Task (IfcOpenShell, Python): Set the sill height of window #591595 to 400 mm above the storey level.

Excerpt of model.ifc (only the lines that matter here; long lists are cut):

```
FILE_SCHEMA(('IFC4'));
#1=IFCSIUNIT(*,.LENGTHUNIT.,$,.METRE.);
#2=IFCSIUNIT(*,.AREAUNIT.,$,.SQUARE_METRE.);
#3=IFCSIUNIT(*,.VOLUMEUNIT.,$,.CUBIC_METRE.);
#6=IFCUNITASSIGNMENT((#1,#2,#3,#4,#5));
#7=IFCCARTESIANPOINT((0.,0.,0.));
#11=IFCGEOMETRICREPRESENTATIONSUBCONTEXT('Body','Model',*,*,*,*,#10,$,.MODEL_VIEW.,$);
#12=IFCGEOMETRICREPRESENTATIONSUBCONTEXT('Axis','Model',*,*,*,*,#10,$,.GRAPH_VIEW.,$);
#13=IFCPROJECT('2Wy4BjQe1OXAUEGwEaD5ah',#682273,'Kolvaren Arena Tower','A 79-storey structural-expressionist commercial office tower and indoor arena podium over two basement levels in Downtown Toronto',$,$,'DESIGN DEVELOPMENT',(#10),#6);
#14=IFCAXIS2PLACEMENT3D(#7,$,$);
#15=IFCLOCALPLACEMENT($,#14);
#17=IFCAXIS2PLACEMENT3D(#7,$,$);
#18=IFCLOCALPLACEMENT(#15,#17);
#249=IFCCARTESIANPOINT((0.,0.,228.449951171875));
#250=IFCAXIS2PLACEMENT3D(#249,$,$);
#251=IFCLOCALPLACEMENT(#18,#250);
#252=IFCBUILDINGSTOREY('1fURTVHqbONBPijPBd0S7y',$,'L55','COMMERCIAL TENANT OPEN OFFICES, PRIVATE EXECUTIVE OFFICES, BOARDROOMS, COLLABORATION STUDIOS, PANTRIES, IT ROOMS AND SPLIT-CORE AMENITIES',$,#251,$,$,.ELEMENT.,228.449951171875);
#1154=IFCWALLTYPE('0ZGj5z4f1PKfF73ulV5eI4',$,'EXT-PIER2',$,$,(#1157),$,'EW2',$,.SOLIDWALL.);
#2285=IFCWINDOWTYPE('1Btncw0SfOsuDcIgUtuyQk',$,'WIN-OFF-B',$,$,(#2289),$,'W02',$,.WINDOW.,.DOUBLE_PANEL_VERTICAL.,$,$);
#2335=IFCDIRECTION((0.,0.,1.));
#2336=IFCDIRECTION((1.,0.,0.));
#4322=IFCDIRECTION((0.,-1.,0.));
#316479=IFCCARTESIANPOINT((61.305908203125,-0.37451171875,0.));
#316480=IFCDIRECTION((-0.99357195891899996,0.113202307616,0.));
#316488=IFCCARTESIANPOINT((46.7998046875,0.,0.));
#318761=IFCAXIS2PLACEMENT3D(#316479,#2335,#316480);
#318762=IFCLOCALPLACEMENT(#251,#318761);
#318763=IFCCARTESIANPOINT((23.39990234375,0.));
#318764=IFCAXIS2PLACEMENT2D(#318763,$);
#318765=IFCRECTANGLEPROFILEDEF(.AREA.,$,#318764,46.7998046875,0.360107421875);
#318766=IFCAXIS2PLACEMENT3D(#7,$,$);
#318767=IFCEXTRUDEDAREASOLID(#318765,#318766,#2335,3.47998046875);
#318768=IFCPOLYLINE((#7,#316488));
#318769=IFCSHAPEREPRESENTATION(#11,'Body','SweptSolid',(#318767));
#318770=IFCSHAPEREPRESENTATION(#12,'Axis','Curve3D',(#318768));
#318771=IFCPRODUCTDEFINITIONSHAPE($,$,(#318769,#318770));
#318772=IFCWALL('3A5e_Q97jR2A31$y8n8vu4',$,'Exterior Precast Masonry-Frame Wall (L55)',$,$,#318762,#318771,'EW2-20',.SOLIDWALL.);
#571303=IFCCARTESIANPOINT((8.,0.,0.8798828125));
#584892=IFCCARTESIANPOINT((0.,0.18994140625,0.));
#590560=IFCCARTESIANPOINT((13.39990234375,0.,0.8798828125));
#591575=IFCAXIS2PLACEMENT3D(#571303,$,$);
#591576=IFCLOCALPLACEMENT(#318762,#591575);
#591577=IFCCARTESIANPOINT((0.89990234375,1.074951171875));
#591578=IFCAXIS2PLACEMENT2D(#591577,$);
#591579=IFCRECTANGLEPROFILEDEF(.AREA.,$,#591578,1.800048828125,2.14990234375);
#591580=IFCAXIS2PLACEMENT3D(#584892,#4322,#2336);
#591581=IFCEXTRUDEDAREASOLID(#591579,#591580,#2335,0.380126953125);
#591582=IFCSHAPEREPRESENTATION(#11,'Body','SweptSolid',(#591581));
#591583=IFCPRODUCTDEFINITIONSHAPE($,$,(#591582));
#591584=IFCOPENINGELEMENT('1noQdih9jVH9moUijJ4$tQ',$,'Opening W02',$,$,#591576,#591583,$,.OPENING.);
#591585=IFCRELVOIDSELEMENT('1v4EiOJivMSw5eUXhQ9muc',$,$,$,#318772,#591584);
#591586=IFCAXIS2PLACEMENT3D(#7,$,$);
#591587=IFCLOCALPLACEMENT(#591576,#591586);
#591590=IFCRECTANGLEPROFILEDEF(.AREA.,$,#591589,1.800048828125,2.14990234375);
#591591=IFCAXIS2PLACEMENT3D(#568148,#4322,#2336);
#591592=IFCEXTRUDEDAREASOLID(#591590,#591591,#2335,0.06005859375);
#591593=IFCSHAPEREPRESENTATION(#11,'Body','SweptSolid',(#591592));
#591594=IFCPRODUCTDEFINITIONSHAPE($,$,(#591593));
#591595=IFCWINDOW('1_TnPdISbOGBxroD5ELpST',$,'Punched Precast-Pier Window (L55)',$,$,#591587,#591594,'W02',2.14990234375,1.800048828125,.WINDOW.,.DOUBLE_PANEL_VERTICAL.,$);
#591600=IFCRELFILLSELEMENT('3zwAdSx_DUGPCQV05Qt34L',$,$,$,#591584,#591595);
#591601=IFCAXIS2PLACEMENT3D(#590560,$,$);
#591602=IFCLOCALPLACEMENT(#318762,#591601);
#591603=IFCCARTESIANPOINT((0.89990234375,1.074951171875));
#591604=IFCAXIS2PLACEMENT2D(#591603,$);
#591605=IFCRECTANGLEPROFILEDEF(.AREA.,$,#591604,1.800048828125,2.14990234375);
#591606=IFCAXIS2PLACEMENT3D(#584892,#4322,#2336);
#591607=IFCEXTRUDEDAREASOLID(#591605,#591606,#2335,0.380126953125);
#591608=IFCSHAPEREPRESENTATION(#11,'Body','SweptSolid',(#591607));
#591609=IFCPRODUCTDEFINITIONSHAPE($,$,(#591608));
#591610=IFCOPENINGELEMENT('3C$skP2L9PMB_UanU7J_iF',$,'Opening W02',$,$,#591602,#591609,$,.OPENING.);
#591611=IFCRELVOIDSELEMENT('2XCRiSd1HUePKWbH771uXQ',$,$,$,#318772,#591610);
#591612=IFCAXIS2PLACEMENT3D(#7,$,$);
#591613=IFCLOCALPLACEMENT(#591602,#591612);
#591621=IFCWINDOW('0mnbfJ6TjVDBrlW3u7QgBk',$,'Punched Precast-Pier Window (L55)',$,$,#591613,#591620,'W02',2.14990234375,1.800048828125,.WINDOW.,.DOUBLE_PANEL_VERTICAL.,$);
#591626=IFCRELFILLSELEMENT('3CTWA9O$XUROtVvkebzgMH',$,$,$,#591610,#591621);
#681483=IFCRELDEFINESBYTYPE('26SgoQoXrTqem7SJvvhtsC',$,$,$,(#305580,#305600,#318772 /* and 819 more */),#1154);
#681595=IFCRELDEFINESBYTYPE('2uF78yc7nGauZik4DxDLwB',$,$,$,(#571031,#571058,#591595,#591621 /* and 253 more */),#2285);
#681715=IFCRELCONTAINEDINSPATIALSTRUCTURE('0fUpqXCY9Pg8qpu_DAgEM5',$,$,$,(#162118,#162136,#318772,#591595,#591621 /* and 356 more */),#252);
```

```python
import numpy as np
import ifcopenshell
import ifcopenshell.api.geometry
import ifcopenshell.geom
import ifcopenshell.util.element
import ifcopenshell.util.placement
import ifcopenshell.util.shape
import ifcopenshell.util.unit

model = ifcopenshell.open("model.ifc")
unit_scale = ifcopenshell.util.unit.calculate_unit_scale(model)

window = model.by_guid("1_TnPdISbOGBxroD5ELpST")
opening = window.FillsVoids[0].RelatingOpeningElement
storey = ifcopenshell.util.element.get_container(window, ifc_class="IfcBuildingStorey")
level = ifcopenshell.util.placement.get_local_placement(storey.ObjectPlacement)[2, 3]

# The opening's origin need not be at the sill, so measure its lowest point.
shape = ifcopenshell.geom.create_shape(ifcopenshell.geom.settings(), opening)
bottom = ifcopenshell.util.shape.get_shape_bottom_elevation(shape, shape.geometry) / unit_scale
dz = level + 0.4 - bottom

shift = np.array([0.0, 0.0, dz])
# The window is placed relative to its opening, so it follows when the opening moves.
matrix = ifcopenshell.util.placement.get_local_placement(opening.ObjectPlacement)
matrix[:3, 3] += shift
ifcopenshell.api.geometry.edit_object_placement(
    model, product=opening, matrix=matrix, is_si=False, should_transform_children=True
)

print(f"moved by {dz * unit_scale:+.3f} m")

model.write("model_v2.ifc")
```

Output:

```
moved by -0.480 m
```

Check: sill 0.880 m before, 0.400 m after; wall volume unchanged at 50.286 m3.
